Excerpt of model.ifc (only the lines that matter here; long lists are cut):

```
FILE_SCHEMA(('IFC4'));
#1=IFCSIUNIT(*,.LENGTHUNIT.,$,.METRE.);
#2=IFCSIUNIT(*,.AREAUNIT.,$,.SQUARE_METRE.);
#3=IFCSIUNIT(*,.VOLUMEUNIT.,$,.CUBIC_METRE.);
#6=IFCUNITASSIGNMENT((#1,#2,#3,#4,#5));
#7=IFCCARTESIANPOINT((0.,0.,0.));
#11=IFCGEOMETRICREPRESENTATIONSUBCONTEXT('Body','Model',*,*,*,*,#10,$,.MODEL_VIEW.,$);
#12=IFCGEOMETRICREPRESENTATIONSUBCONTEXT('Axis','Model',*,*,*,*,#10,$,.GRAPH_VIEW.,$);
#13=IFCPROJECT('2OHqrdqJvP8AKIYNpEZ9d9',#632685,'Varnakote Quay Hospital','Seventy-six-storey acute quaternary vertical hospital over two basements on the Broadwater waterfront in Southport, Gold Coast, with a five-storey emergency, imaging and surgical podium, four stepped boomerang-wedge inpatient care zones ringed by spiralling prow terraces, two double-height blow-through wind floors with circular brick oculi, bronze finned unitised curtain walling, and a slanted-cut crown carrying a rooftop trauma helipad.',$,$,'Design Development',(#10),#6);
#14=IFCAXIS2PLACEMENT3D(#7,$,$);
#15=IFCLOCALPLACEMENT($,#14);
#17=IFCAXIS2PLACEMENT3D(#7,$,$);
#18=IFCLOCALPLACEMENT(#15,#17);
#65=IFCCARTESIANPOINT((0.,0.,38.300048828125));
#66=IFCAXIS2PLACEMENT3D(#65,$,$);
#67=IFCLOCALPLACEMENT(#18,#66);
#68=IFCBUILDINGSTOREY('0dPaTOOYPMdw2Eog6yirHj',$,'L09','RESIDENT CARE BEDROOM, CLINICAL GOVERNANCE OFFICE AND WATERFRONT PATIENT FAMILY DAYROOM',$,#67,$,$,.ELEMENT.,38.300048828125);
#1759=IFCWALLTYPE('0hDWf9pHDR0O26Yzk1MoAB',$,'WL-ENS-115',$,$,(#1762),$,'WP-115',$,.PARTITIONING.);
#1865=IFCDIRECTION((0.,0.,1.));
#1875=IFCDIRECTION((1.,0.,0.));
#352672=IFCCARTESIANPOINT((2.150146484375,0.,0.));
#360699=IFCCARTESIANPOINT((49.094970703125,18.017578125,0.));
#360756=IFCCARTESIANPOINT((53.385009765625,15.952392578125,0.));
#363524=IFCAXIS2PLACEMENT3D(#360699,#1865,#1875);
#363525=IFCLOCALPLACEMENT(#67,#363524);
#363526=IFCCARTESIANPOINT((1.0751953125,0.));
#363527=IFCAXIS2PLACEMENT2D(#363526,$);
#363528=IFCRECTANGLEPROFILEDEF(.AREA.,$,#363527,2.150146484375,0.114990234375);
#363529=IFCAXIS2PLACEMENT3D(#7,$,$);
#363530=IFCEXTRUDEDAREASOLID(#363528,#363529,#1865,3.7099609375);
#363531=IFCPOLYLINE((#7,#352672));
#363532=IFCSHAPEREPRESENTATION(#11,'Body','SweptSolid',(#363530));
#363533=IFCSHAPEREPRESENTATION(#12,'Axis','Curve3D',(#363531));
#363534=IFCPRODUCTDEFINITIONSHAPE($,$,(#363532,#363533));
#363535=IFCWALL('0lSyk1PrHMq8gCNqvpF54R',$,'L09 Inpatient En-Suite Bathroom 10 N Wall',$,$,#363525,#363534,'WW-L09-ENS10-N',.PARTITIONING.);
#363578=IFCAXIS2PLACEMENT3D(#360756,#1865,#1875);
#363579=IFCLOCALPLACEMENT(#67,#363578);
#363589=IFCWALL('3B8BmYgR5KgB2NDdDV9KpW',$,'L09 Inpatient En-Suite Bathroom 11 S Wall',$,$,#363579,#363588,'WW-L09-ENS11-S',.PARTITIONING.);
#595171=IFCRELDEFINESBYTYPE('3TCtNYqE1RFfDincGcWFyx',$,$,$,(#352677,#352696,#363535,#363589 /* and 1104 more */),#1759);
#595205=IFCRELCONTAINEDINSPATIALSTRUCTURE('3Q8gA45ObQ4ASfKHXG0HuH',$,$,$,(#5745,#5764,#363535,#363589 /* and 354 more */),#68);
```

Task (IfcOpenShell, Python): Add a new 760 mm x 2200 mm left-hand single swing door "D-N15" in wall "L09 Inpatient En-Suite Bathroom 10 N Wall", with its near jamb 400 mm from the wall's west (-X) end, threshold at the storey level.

```python
import numpy as np
import ifcopenshell
import ifcopenshell.api.feature
import ifcopenshell.api.geometry
import ifcopenshell.api.root
import ifcopenshell.api.spatial
import ifcopenshell.geom
import ifcopenshell.util.element
import ifcopenshell.util.placement
import ifcopenshell.util.representation
import ifcopenshell.util.shape
import ifcopenshell.util.unit

model = ifcopenshell.open("model.ifc")
unit_scale = ifcopenshell.util.unit.calculate_unit_scale(model)
settings = ifcopenshell.geom.settings()


def volume(element):
    """Net volume in cubic metres, openings subtracted."""
    shape = ifcopenshell.geom.create_shape(settings, element)
    return ifcopenshell.util.shape.get_volume(shape.geometry)


wall = model.by_id(363535)
storey = ifcopenshell.util.element.get_container(wall, ifc_class="IfcBuildingStorey")
context = ifcopenshell.util.representation.get_context(model, "Model", "Body", "MODEL_VIEW")
before = volume(wall)

width, height, from_end, sill = 0.76, 2.2, 0.4, 0.0  # metres

# The wall runs along its own X axis, and the end named is its -X end.
wall_shape = ifcopenshell.geom.create_shape(settings, wall)
x, y, z = ifcopenshell.util.shape.get_vertices(wall_shape.geometry).T
start = x.min() + from_end
face, thickness = float(y.min()), float(y.max() - y.min())
wall_matrix = ifcopenshell.util.placement.get_local_placement(wall.ObjectPlacement)
level = ifcopenshell.util.placement.get_local_placement(storey.ObjectPlacement)[2, 3]


def in_wall(x, y):
    """Placement at x, y metres in the wall's axes, at sill height."""
    matrix = wall_matrix.copy()
    matrix[:, 3] = wall_matrix @ np.array([x / unit_scale, y / unit_scale, 0.0, 1.0])
    matrix[2, 3] = level + sill / unit_scale
    return matrix


# Opening: a box that overshoots both wall faces by 50 mm.
opening = ifcopenshell.api.root.create_entity(model, ifc_class="IfcOpeningElement", predefined_type="OPENING")
box = ifcopenshell.api.geometry.add_wall_representation(
    model, context=context, length=width, height=height, thickness=thickness + 0.1
)
ifcopenshell.api.geometry.assign_representation(model, product=opening, representation=box)
ifcopenshell.api.geometry.edit_object_placement(model, product=opening, matrix=in_wall(start, face - 0.05), is_si=False)
ifcopenshell.api.feature.add_feature(model, feature=opening, element=wall)

door = ifcopenshell.api.root.create_entity(model, ifc_class="IfcDoor", name="D-N15", predefined_type="DOOR")
door.OverallWidth, door.OverallHeight = width / unit_scale, height / unit_scale
door.OperationType = "SINGLE_SWING_LEFT"
body = ifcopenshell.api.geometry.add_door_representation(
    model,
    context=context,
    overall_width=door.OverallWidth,
    overall_height=door.OverallHeight,
    operation_type="SINGLE_SWING_LEFT",
    lining_properties={"LiningDepth": thickness / unit_scale, "ThresholdDepth": thickness / unit_scale},
)
ifcopenshell.api.geometry.assign_representation(model, product=door, representation=body)
ifcopenshell.api.spatial.assign_container(model, products=[door], relating_structure=storey)
ifcopenshell.api.feature.add_filling(model, opening=opening, element=door)

# The lining spans the wall, so the door starts at the wall face.
ifcopenshell.api.geometry.edit_object_placement(model, product=door, matrix=in_wall(start, face), is_si=False)

after = volume(wall)

print(f"wall volume {before:.3f} -> {after:.3f} m3")

model.write("model-out.ifc")
```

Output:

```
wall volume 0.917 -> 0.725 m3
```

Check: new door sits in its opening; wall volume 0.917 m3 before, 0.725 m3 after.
